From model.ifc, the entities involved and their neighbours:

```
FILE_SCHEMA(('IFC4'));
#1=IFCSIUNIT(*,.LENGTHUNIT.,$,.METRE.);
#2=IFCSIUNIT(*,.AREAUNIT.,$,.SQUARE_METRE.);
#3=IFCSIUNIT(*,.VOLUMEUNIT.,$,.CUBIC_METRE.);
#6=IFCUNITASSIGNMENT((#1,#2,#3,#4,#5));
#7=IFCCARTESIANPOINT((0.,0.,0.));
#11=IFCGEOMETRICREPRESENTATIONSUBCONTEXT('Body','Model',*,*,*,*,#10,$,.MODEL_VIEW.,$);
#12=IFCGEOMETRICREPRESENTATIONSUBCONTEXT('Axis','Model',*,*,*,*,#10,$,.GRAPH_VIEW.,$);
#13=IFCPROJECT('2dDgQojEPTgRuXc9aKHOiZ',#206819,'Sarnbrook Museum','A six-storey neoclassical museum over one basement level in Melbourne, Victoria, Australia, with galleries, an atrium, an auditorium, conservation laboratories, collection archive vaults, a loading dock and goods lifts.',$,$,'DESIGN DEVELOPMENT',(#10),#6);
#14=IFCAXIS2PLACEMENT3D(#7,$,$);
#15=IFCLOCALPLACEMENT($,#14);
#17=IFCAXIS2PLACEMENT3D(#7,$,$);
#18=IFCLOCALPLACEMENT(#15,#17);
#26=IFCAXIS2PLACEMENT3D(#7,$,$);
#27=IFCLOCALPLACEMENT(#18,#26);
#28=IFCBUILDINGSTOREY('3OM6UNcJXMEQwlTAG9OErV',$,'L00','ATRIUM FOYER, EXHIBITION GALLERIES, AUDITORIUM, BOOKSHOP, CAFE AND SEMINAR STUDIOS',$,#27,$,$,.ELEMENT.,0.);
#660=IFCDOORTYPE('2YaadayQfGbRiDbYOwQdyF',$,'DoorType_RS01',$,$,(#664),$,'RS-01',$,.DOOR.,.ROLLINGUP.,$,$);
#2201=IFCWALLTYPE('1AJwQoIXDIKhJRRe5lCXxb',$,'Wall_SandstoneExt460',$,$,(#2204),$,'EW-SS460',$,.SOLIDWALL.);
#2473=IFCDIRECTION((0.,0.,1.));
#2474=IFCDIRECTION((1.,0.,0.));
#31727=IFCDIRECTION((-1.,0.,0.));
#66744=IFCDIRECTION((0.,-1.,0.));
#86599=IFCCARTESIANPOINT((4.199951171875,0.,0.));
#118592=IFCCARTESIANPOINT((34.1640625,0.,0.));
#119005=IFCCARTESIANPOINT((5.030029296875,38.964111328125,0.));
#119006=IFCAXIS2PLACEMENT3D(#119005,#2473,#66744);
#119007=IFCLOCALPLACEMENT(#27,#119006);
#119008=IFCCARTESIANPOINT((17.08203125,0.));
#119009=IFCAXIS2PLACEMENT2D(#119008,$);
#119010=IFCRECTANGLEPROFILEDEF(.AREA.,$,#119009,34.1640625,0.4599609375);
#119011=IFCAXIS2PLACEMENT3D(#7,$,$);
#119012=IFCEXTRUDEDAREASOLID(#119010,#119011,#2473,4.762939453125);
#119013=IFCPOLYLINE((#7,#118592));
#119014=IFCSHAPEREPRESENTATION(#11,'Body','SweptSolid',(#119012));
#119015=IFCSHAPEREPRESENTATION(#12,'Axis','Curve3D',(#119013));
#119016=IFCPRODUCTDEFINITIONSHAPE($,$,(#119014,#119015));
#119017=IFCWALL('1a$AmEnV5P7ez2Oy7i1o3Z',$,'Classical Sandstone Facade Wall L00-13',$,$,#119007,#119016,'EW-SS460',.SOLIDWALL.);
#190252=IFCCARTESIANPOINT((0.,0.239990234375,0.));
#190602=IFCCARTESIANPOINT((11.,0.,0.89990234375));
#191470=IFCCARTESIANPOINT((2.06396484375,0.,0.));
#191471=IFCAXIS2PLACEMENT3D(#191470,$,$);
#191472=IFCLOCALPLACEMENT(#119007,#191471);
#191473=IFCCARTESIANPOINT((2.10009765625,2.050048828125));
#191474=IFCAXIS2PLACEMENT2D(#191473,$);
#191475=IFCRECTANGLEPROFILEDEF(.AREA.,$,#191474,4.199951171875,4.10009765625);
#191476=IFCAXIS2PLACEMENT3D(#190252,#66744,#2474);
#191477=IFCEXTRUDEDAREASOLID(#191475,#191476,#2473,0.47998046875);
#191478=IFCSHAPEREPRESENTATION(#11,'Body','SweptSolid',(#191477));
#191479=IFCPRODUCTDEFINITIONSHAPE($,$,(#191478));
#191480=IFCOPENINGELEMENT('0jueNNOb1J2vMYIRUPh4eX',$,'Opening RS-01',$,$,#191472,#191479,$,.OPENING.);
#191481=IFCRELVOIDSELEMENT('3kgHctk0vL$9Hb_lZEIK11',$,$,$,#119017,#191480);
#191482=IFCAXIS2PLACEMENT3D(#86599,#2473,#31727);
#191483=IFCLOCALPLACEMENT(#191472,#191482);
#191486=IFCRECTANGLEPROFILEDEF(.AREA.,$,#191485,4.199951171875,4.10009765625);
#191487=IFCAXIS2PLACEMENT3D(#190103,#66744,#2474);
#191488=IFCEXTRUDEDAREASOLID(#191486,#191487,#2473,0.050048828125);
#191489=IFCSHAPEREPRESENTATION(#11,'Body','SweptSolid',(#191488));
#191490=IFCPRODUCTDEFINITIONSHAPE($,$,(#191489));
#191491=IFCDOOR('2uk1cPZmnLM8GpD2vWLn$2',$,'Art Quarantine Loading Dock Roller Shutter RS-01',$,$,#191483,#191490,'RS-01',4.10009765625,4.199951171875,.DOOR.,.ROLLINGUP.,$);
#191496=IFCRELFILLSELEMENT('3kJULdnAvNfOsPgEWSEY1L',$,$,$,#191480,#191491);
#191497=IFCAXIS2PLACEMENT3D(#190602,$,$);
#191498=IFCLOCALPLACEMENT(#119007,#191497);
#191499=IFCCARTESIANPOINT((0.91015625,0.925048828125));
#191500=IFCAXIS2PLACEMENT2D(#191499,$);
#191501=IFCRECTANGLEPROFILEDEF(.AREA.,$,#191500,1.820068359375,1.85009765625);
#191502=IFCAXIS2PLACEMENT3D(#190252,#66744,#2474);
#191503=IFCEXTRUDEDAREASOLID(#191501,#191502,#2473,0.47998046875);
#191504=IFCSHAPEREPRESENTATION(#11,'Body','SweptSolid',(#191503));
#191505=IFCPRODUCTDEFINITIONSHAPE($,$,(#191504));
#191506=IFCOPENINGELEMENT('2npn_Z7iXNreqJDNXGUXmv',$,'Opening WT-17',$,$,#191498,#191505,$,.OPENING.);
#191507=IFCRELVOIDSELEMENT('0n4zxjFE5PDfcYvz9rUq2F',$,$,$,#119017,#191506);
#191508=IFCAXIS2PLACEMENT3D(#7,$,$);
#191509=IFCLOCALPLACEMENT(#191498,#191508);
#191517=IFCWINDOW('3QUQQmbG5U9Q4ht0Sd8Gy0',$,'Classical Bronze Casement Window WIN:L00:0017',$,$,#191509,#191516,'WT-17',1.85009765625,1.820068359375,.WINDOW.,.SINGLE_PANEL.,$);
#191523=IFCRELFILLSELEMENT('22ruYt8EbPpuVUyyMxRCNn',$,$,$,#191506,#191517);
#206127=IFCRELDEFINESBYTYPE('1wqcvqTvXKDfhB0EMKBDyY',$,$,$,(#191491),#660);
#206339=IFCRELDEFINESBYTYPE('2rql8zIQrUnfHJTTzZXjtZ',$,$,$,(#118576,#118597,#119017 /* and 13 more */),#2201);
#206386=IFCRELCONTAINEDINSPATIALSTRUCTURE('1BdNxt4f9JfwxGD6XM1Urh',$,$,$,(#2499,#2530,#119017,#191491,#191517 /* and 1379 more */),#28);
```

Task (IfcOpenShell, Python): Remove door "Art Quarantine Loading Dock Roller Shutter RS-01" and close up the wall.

```python
import ifcopenshell
import ifcopenshell.api.feature
import ifcopenshell.api.root
import ifcopenshell.geom
import ifcopenshell.util.shape

model = ifcopenshell.open("model.ifc")
settings = ifcopenshell.geom.settings()


def volume(element):
    """Net volume in cubic metres, openings subtracted."""
    shape = ifcopenshell.geom.create_shape(settings, element)
    return ifcopenshell.util.shape.get_volume(shape.geometry)


door = model.by_guid("2uk1cPZmnLM8GpD2vWLn$2")
opening = door.FillsVoids[0].RelatingOpeningElement
wall = opening.VoidsElements[0].RelatingBuildingElement
before = volume(wall)

ifcopenshell.api.root.remove_product(model, product=door)
ifcopenshell.api.feature.remove_feature(model, feature=opening)

after = volume(wall)

print(f"wall volume {before:.3f} -> {after:.3f} m3")

model.write("model_edited.ifc")
```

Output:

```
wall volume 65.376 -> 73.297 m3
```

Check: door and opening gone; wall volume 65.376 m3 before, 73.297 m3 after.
